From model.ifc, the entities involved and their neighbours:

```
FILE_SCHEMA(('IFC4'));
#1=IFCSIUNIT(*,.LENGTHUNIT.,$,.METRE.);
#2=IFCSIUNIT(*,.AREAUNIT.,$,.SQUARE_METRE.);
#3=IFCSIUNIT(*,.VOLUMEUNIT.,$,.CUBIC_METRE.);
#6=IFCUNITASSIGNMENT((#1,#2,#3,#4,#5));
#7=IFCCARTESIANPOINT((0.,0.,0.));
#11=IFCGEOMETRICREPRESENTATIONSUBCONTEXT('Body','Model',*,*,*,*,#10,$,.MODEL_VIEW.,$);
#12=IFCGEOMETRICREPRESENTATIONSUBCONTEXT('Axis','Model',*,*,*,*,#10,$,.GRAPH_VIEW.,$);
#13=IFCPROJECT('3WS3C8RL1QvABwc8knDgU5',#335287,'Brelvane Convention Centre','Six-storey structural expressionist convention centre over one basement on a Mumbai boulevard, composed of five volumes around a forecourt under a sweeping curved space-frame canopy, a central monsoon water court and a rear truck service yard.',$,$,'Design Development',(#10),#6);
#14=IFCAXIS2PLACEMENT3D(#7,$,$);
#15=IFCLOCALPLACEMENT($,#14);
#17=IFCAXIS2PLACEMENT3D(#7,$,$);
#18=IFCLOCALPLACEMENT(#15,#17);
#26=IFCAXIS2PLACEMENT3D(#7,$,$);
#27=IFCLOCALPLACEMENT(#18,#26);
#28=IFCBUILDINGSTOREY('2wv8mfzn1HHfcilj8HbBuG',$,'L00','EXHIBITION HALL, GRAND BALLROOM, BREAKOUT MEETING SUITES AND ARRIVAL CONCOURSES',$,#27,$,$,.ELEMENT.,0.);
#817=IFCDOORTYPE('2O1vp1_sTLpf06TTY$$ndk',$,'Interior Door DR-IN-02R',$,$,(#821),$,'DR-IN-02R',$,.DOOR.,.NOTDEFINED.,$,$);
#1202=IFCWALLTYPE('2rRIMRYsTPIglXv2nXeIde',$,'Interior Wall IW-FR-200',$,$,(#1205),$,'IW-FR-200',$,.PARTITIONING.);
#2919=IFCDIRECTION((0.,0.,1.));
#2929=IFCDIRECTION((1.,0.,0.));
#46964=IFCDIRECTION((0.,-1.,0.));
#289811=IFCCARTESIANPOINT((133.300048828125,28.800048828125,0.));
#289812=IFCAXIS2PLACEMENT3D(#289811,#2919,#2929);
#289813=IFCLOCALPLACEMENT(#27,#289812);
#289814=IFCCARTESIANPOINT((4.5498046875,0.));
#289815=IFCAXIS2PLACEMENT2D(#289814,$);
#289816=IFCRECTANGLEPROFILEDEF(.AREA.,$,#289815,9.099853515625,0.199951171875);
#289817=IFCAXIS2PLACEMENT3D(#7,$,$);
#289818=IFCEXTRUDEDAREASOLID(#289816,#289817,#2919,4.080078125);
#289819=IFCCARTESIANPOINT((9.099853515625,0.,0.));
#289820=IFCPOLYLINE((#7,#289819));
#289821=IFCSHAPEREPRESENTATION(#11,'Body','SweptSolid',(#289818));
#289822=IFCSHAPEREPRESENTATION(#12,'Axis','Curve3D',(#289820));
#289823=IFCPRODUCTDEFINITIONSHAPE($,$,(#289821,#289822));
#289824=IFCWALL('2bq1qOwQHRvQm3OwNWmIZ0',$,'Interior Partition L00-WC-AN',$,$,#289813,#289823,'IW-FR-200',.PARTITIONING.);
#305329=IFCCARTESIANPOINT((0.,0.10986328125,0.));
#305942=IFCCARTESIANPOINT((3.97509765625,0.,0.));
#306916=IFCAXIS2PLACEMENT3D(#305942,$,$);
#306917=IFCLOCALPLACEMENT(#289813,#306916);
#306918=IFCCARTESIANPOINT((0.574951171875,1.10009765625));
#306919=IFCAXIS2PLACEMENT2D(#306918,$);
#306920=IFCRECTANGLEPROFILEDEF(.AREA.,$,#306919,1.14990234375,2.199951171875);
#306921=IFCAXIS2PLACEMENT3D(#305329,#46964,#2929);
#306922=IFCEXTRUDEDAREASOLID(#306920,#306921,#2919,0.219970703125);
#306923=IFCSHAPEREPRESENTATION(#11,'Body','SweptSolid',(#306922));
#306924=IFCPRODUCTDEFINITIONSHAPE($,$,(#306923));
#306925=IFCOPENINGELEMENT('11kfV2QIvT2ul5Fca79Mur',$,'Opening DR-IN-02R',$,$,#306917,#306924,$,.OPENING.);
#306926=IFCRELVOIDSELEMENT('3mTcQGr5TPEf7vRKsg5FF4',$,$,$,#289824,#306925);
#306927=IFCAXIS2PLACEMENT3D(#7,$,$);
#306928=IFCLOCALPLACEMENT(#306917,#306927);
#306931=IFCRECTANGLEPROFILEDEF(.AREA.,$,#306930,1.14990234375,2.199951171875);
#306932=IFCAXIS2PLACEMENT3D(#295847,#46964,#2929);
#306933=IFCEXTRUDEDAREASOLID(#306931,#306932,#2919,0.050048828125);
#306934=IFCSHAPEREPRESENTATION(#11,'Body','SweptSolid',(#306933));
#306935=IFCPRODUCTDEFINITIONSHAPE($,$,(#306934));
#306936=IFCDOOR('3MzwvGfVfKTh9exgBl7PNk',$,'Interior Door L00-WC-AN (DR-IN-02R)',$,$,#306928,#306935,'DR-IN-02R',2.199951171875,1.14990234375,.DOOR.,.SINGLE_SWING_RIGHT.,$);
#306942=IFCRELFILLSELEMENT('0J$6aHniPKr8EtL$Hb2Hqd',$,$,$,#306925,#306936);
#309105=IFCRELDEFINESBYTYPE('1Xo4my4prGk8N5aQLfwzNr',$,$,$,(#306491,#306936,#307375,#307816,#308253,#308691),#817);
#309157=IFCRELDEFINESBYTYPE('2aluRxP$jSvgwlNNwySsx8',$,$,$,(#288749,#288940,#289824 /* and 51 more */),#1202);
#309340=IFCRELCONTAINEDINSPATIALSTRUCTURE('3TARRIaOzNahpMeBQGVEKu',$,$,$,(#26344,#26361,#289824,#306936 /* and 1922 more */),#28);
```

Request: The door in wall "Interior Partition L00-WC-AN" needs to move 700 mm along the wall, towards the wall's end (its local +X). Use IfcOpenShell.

```python
import ifcopenshell
import ifcopenshell.api.geometry
import ifcopenshell.util.placement
import ifcopenshell.util.unit

model = ifcopenshell.open("model.ifc")
unit_scale = ifcopenshell.util.unit.calculate_unit_scale(model)

door = model.by_guid("3MzwvGfVfKTh9exgBl7PNk")
opening = door.FillsVoids[0].RelatingOpeningElement
wall = opening.VoidsElements[0].RelatingBuildingElement

wall_matrix = ifcopenshell.util.placement.get_local_placement(wall.ObjectPlacement)
shift = wall_matrix[:3, 0] * 0.7 / unit_scale
before = ifcopenshell.util.placement.get_local_placement(door.ObjectPlacement)[:3, 3].copy()

# The door is placed relative to its opening, so it follows when the opening moves.
matrix = ifcopenshell.util.placement.get_local_placement(opening.ObjectPlacement)
matrix[:3, 3] += shift
ifcopenshell.api.geometry.edit_object_placement(
    model, product=opening, matrix=matrix, is_si=False, should_transform_children=True
)

after = ifcopenshell.util.placement.get_local_placement(door.ObjectPlacement)[:3, 3]
print("door moved by", (after - before).round(3) + 0.0)

model.write("model_v2.ifc")
```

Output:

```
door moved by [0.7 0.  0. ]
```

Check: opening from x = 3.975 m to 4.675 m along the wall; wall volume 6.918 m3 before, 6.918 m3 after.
